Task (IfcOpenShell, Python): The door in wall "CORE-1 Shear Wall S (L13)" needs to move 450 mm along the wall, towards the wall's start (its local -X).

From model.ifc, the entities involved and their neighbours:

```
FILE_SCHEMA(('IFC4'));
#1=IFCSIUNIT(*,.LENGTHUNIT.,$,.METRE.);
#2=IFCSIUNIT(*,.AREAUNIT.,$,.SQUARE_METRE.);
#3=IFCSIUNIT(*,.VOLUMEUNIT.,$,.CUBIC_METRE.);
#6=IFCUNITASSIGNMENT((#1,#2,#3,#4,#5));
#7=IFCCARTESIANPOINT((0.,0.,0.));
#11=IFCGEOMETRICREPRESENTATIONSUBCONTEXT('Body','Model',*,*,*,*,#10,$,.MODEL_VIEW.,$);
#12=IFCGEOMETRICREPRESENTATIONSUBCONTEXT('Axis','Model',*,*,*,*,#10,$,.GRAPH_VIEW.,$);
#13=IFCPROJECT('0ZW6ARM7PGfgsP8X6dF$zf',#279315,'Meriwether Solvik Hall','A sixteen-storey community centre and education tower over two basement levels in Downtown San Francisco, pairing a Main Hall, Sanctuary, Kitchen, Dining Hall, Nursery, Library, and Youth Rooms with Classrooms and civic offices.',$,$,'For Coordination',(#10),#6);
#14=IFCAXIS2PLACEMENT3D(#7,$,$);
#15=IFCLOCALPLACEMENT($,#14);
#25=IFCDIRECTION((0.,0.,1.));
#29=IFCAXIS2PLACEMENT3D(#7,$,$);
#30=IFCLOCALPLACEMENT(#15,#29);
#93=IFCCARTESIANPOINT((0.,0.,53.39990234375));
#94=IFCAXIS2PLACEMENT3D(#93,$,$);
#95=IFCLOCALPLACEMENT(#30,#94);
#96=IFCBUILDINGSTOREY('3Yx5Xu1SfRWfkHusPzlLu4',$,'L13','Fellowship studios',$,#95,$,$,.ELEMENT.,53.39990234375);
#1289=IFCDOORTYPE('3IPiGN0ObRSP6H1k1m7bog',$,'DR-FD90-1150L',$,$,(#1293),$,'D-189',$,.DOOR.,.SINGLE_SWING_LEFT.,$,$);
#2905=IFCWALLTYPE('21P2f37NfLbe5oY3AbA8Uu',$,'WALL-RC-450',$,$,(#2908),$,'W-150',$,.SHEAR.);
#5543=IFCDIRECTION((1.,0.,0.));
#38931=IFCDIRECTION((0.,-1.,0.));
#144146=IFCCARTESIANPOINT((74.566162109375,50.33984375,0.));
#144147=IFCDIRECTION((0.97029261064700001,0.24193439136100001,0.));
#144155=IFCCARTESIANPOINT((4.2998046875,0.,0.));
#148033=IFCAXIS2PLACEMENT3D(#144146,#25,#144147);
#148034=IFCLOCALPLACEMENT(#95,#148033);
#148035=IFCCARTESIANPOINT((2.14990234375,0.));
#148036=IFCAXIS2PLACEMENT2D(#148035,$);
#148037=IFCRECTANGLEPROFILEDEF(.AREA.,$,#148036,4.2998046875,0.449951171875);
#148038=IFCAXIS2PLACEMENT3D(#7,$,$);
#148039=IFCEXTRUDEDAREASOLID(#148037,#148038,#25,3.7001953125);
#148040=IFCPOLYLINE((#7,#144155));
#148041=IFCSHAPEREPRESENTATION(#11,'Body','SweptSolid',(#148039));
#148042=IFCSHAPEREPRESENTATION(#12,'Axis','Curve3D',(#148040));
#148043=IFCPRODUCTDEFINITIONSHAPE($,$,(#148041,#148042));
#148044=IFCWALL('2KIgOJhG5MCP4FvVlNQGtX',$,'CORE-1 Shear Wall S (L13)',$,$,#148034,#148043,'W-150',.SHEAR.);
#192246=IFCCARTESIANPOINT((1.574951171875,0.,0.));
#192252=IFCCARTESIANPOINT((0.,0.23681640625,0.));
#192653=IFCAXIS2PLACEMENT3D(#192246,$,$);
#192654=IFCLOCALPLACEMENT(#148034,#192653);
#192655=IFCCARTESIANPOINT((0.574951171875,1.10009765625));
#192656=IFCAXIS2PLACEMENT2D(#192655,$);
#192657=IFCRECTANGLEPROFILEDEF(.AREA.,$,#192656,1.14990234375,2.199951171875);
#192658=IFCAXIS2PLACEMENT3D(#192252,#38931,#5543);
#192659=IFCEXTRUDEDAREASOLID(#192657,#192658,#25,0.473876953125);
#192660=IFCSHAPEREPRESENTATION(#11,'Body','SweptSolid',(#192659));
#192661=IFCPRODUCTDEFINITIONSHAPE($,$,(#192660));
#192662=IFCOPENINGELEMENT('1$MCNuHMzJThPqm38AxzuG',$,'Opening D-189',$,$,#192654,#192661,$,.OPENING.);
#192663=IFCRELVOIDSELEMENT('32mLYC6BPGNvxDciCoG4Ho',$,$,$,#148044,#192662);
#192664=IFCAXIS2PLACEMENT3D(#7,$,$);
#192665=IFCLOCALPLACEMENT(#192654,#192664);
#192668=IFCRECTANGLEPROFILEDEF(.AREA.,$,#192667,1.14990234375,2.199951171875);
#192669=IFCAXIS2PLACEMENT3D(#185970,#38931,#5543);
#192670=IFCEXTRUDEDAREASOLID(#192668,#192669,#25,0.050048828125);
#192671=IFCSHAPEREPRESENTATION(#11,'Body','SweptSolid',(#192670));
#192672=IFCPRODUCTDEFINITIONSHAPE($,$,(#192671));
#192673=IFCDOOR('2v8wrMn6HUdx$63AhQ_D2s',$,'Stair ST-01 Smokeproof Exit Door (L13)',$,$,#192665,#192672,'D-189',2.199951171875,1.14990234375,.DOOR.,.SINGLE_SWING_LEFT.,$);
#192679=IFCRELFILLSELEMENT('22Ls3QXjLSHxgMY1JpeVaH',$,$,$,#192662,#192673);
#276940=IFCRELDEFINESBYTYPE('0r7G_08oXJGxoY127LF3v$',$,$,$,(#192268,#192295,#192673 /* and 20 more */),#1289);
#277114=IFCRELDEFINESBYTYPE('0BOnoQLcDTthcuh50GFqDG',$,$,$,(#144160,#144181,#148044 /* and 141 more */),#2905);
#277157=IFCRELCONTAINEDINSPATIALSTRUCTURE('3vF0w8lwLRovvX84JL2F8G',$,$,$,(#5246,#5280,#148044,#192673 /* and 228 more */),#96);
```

```python
import ifcopenshell
import ifcopenshell.api.geometry
import ifcopenshell.util.placement

model = ifcopenshell.open("model.ifc")

door = model.by_id(192673)
opening = door.FillsVoids[0].RelatingOpeningElement
wall = opening.VoidsElements[0].RelatingBuildingElement

wall_matrix = ifcopenshell.util.placement.get_local_placement(wall.ObjectPlacement)
shift = wall_matrix[:3, 0] * -0.45
before = ifcopenshell.util.placement.get_local_placement(door.ObjectPlacement)[:3, 3].copy()

# The door is placed relative to its opening, so it follows when the opening moves.
matrix = ifcopenshell.util.placement.get_local_placement(opening.ObjectPlacement)
matrix[:3, 3] += shift
ifcopenshell.api.geometry.edit_object_placement(
    model, product=opening, matrix=matrix, is_si=False, should_transform_children=True
)

after = ifcopenshell.util.placement.get_local_placement(door.ObjectPlacement)[:3, 3]
print("door moved by", (after - before).round(3) + 0.0)

model.write("model_v2.ifc")
```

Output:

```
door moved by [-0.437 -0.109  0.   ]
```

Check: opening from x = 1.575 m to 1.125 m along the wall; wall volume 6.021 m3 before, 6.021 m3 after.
